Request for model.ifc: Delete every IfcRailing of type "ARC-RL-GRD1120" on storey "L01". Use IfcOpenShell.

First a look at what the model holds.

```python
import ifcopenshell
import ifcopenshell.util.element

model = ifcopenshell.open("model.ifc")
print(model.schema)
storey = next(s for s in model.by_type("IfcBuildingStorey") if s.Name == "L01")
railings = [e for e in ifcopenshell.util.element.get_decomposition(storey) if e.is_a("IfcRailing")]
seen = {}
for e in railings:
    element_type = ifcopenshell.util.element.get_type(e)
    name = element_type.Name if element_type not in (None, e) else None
    seen[name] = seen.get(name, 0) + 1
for name, count in sorted(seen.items(), key=str):
    print(count, "x", name)
```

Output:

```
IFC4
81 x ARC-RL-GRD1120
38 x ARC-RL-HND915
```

```python
import ifcopenshell
import ifcopenshell.api.root
import ifcopenshell.util.element

model = ifcopenshell.open("model.ifc")

storey = next(s for s in model.by_type("IfcBuildingStorey") if s.Name == "L01")
railings = [e for e in ifcopenshell.util.element.get_decomposition(storey) if e.is_a("IfcRailing")]
targets = [e for e in railings if (t := ifcopenshell.util.element.get_type(e)) not in (None, e) and t.Name == "ARC-RL-GRD1120"]

for e in targets:
    ifcopenshell.api.root.remove_product(model, product=e)
print(len(targets), "removed")

model.write("model-out.ifc")
```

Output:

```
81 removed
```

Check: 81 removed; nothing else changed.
